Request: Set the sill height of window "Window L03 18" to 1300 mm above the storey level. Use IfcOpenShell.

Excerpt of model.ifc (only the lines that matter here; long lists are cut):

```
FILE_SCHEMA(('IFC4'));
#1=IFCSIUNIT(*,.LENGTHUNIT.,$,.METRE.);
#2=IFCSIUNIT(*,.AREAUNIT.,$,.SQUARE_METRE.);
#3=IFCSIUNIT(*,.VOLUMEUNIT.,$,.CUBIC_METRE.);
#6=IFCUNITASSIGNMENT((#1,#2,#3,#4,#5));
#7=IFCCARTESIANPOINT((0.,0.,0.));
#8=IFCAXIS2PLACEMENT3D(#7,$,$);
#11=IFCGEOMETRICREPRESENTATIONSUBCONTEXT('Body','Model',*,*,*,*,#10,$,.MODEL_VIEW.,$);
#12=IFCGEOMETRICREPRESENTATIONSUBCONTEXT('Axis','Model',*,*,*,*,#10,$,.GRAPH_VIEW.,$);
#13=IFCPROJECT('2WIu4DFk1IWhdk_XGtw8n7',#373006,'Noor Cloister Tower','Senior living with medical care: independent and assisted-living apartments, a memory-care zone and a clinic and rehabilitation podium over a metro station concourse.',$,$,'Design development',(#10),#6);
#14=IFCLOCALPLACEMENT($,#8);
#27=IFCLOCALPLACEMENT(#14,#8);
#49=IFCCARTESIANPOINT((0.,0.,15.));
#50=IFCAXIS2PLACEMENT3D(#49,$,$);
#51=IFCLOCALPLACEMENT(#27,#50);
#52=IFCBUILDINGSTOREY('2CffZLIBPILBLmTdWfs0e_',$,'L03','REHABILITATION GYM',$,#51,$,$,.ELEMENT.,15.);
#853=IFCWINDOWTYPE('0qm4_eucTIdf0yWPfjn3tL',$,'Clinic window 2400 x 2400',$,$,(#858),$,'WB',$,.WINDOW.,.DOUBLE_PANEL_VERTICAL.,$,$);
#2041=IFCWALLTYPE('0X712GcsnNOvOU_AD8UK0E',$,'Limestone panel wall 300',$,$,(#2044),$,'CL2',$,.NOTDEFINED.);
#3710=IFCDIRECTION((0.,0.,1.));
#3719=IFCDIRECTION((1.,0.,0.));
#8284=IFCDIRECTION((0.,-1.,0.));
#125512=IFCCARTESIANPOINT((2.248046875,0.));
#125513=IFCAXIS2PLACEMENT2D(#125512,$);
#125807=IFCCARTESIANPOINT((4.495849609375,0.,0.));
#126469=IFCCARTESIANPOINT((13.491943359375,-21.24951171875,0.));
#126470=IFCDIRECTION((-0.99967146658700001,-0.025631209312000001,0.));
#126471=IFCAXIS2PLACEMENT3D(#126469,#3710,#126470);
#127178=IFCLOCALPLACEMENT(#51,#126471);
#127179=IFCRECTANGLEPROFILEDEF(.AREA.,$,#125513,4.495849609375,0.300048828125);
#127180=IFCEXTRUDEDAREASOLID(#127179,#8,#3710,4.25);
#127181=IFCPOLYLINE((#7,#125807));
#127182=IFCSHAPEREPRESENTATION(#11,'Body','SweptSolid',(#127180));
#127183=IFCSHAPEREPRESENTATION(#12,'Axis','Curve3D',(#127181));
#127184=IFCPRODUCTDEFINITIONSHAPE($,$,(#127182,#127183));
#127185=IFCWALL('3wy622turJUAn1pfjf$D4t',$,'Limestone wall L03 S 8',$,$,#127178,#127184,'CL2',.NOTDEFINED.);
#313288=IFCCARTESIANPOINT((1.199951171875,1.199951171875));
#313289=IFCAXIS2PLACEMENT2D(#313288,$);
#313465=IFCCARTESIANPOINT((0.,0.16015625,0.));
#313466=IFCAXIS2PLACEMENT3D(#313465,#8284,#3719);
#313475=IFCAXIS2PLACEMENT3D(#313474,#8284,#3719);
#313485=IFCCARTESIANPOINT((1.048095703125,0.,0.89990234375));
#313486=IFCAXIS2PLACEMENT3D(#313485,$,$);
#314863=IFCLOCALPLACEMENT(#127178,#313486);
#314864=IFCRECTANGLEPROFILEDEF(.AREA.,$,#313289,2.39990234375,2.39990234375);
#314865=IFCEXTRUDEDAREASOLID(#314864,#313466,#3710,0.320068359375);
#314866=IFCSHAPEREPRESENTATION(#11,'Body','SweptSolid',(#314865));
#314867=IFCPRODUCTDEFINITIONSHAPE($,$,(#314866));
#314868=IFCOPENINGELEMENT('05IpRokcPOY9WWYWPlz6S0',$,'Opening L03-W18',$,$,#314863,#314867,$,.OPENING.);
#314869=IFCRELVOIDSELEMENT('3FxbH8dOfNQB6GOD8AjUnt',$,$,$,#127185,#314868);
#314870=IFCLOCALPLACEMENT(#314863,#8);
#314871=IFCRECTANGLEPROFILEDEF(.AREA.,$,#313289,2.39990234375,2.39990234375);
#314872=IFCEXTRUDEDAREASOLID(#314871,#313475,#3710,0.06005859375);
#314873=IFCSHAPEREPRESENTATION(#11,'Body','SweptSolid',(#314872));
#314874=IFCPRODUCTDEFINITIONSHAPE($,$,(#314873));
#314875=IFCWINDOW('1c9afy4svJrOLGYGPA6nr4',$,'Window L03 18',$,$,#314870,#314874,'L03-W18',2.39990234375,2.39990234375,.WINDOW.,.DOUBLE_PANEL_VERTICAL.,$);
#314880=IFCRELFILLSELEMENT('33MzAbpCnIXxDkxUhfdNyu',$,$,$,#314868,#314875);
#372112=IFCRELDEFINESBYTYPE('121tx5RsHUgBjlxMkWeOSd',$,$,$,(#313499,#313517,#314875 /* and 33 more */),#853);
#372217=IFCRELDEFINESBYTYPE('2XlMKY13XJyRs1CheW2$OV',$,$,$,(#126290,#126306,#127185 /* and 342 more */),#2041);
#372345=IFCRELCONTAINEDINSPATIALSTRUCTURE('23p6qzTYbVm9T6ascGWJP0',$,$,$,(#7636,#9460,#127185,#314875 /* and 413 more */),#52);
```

```python
import numpy as np
import ifcopenshell
import ifcopenshell.api.geometry
import ifcopenshell.geom
import ifcopenshell.util.element
import ifcopenshell.util.placement
import ifcopenshell.util.shape
import ifcopenshell.util.unit

model = ifcopenshell.open("model.ifc")
unit_scale = ifcopenshell.util.unit.calculate_unit_scale(model)

window = model.by_guid("1c9afy4svJrOLGYGPA6nr4")
opening = window.FillsVoids[0].RelatingOpeningElement
storey = ifcopenshell.util.element.get_container(window, ifc_class="IfcBuildingStorey")
level = ifcopenshell.util.placement.get_local_placement(storey.ObjectPlacement)[2, 3]

# The opening's origin need not be at the sill, so measure its lowest point.
shape = ifcopenshell.geom.create_shape(ifcopenshell.geom.settings(), opening)
bottom = ifcopenshell.util.shape.get_shape_bottom_elevation(shape, shape.geometry) / unit_scale
dz = level + 1.3 / unit_scale - bottom

shift = np.array([0.0, 0.0, dz])
# The window is placed relative to its opening, so it follows when the opening moves.
matrix = ifcopenshell.util.placement.get_local_placement(opening.ObjectPlacement)
matrix[:3, 3] += shift
ifcopenshell.api.geometry.edit_object_placement(
    model, product=opening, matrix=matrix, is_si=False, should_transform_children=True
)

print(f"moved by {dz * unit_scale:+.3f} m")

model.write("model-out.ifc")
```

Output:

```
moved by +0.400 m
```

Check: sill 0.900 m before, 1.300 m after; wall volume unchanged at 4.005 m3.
